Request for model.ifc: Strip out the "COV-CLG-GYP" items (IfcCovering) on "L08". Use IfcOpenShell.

First a look at what the model holds.

```python
import ifcopenshell
import ifcopenshell.util.element

model = ifcopenshell.open("model.ifc")
print(model.schema)
storey = next(s for s in model.by_type("IfcBuildingStorey") if s.Name == "L08")
coverings = [e for e in ifcopenshell.util.element.get_decomposition(storey) if e.is_a("IfcCovering")]
seen = {}
for e in coverings:
    element_type = ifcopenshell.util.element.get_type(e)
    name = element_type.Name if element_type not in (None, e) else None
    seen[name] = seen.get(name, 0) + 1
for name, count in sorted(seen.items(), key=str):
    print(count, "x", name)
```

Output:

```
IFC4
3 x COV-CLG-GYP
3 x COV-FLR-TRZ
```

```python
import ifcopenshell
import ifcopenshell.api.root
import ifcopenshell.util.element

model = ifcopenshell.open("model.ifc")

storey = next(s for s in model.by_type("IfcBuildingStorey") if s.Name == "L08")
coverings = [e for e in ifcopenshell.util.element.get_decomposition(storey) if e.is_a("IfcCovering")]
targets = [e for e in coverings if (t := ifcopenshell.util.element.get_type(e)) not in (None, e) and t.Name == "COV-CLG-GYP"]

for e in targets:
    ifcopenshell.api.root.remove_product(model, product=e)
print(len(targets), "removed")

model.write("model_updated.ifc")
```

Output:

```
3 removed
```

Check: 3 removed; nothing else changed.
